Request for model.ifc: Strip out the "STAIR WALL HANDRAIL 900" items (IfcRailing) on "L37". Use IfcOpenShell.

First a look at what the model holds.

```python
import ifcopenshell
import ifcopenshell.util.element

model = ifcopenshell.open("model.ifc")
print(model.schema)
storey = next(s for s in model.by_type("IfcBuildingStorey") if s.Name == "L37")
railings = [e for e in ifcopenshell.util.element.get_decomposition(storey) if e.is_a("IfcRailing")]
seen = {}
for e in railings:
    element_type = ifcopenshell.util.element.get_type(e)
    name = element_type.Name if element_type not in (None, e) else None
    seen[name] = seen.get(name, 0) + 1
for name, count in sorted(seen.items(), key=str):
    print(count, "x", name)
```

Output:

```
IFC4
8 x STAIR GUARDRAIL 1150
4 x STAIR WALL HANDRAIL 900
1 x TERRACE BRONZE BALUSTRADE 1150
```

```python
import ifcopenshell
import ifcopenshell.api.root
import ifcopenshell.util.element

model = ifcopenshell.open("model.ifc")

storey = next(s for s in model.by_type("IfcBuildingStorey") if s.Name == "L37")
railings = [e for e in ifcopenshell.util.element.get_decomposition(storey) if e.is_a("IfcRailing")]
targets = [e for e in railings if (t := ifcopenshell.util.element.get_type(e)) not in (None, e) and t.Name == "STAIR WALL HANDRAIL 900"]

for e in targets:
    ifcopenshell.api.root.remove_product(model, product=e)
print(len(targets), "removed")

model.write("model_v2.ifc")
```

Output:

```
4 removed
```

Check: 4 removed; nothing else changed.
